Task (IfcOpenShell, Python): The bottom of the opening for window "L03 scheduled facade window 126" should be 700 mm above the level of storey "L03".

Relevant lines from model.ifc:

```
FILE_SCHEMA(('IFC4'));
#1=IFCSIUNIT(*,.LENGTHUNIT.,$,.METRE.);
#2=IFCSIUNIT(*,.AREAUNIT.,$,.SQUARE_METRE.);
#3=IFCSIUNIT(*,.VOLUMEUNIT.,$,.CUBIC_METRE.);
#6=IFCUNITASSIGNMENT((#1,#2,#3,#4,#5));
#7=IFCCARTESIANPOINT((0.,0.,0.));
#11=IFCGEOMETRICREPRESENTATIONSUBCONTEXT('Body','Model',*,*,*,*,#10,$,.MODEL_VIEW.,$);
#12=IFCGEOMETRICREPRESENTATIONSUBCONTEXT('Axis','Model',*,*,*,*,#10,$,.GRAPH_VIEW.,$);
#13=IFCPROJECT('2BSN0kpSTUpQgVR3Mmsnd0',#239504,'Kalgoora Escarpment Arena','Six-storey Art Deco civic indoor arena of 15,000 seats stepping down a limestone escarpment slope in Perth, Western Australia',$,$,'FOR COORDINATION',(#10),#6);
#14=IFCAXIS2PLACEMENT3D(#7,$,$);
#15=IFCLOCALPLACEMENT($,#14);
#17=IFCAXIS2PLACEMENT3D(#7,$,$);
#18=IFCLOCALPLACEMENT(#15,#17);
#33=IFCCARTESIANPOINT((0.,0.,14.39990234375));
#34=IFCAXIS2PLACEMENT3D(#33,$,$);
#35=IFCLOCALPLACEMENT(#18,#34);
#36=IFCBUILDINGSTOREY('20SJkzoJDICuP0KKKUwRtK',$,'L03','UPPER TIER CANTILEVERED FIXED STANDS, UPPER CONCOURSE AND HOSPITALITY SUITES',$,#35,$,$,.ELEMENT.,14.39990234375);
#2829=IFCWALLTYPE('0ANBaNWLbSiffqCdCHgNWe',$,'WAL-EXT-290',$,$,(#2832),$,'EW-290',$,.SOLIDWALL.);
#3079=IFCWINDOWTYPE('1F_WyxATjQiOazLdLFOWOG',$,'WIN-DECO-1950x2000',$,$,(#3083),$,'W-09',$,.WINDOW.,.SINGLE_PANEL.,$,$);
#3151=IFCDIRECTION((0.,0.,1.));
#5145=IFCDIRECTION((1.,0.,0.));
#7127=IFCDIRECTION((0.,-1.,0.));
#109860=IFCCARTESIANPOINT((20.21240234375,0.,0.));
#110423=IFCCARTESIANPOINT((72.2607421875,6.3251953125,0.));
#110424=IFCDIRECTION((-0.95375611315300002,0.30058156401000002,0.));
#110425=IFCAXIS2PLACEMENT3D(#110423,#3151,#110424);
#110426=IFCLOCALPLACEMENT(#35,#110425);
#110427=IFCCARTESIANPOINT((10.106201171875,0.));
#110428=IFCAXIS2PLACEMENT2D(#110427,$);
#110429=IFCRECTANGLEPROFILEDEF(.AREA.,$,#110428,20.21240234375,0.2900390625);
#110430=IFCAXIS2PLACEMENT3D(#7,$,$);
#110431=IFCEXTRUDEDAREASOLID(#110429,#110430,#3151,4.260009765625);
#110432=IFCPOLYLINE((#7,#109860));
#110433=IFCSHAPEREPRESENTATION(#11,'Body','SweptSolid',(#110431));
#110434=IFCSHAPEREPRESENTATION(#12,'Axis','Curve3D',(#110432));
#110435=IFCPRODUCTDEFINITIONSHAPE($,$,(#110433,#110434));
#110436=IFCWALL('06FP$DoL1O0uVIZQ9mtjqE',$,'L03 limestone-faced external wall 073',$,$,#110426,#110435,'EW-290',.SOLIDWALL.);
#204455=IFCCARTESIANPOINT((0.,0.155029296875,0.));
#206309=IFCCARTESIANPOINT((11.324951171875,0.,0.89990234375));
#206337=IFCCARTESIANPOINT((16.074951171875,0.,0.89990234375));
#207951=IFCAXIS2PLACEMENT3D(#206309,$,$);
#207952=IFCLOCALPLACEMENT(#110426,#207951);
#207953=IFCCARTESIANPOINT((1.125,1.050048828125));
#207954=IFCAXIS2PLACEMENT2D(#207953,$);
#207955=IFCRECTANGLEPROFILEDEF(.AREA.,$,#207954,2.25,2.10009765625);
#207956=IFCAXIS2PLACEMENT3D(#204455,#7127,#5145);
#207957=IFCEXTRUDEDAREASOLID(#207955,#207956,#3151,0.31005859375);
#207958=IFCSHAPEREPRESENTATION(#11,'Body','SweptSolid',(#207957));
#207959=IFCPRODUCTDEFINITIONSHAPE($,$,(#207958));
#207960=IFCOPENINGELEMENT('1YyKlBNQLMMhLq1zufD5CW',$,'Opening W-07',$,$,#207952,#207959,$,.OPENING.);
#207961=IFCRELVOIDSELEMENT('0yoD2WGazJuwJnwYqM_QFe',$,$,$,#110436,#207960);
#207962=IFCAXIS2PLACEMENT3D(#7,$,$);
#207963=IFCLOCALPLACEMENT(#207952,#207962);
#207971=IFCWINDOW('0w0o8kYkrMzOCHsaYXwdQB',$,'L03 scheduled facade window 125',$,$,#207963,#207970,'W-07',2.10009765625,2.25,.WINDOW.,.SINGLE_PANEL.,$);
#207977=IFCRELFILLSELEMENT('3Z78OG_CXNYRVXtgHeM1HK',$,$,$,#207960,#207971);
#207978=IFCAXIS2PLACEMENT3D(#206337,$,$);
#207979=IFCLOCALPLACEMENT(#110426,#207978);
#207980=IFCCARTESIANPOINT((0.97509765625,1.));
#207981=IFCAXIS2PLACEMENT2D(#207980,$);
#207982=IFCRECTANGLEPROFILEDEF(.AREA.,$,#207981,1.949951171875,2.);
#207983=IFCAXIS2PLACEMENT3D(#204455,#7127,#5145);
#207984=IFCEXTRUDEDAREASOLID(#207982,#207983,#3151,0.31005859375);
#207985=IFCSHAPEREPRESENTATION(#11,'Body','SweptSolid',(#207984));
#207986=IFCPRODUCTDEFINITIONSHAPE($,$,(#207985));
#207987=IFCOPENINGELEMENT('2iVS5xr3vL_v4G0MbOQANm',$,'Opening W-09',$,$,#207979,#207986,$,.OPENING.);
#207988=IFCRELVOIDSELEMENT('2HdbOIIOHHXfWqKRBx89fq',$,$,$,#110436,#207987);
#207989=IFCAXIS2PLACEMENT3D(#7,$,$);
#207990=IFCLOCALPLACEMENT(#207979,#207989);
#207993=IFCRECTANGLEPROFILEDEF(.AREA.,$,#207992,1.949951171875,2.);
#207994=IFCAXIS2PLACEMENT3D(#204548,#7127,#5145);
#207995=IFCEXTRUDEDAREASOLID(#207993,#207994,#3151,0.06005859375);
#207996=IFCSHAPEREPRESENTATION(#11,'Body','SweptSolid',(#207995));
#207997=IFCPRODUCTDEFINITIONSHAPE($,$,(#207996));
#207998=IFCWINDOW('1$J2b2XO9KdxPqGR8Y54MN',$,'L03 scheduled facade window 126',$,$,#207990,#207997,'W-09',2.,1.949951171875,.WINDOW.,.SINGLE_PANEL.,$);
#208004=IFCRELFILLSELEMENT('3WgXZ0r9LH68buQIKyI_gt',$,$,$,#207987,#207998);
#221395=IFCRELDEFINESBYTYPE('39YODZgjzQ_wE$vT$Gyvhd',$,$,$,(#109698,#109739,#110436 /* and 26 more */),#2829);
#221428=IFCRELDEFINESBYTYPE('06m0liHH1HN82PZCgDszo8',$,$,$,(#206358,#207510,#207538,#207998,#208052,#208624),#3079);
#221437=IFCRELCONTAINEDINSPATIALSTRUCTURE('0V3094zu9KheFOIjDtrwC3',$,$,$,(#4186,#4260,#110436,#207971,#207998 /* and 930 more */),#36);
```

```python
import numpy as np
import ifcopenshell
import ifcopenshell.api.geometry
import ifcopenshell.geom
import ifcopenshell.util.element
import ifcopenshell.util.placement
import ifcopenshell.util.shape
import ifcopenshell.util.unit

model = ifcopenshell.open("model.ifc")
unit_scale = ifcopenshell.util.unit.calculate_unit_scale(model)

window = model.by_guid("1$J2b2XO9KdxPqGR8Y54MN")
opening = window.FillsVoids[0].RelatingOpeningElement
storey = ifcopenshell.util.element.get_container(window, ifc_class="IfcBuildingStorey")
level = ifcopenshell.util.placement.get_local_placement(storey.ObjectPlacement)[2, 3]

# The opening's origin need not be at the sill, so measure its lowest point.
shape = ifcopenshell.geom.create_shape(ifcopenshell.geom.settings(), opening)
bottom = ifcopenshell.util.shape.get_shape_bottom_elevation(shape, shape.geometry) / unit_scale
dz = level + 0.7 / unit_scale - bottom

shift = np.array([0.0, 0.0, dz])
# The window is placed relative to its opening, so it follows when the opening moves.
matrix = ifcopenshell.util.placement.get_local_placement(opening.ObjectPlacement)
matrix[:3, 3] += shift
ifcopenshell.api.geometry.edit_object_placement(
    model, product=opening, matrix=matrix, is_si=False, should_transform_children=True
)

print(f"moved by {dz * unit_scale:+.3f} m")

model.write("model-out.ifc")
```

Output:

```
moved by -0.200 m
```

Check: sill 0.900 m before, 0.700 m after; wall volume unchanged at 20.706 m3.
